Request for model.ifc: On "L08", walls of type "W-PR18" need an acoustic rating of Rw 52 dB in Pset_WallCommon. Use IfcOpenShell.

First a look at what the model holds.

```python
import ifcopenshell
import ifcopenshell.util.element

model = ifcopenshell.open("model.ifc")
print(model.schema)
storey = next(s for s in model.by_type("IfcBuildingStorey") if s.Name == "L08")
walls = [e for e in ifcopenshell.util.element.get_decomposition(storey) if e.is_a("IfcWall")]
seen = {}
for e in walls:
    element_type = ifcopenshell.util.element.get_type(e)
    key = (element_type.Name if element_type != e and element_type else None, ifcopenshell.util.element.get_pset(e, "Pset_WallCommon", "AcousticRating"))
    seen[key] = seen.get(key, 0) + 1
for (name, value), count in sorted(seen.items(), key=str):
    print(count, "x", name, "|", value)
```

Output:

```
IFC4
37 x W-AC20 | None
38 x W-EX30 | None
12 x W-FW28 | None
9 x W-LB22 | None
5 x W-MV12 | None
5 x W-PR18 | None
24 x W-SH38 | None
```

```python
import ifcopenshell
import ifcopenshell.api.pset
import ifcopenshell.util.element

model = ifcopenshell.open("model.ifc")

storey = next(s for s in model.by_type("IfcBuildingStorey") if s.Name == "L08")
walls = [e for e in ifcopenshell.util.element.get_decomposition(storey) if e.is_a("IfcWall")]

count = 0
for e in walls:
    element_type = ifcopenshell.util.element.get_type(e)
    if element_type in (None, e) or element_type.Name != "W-PR18":
        continue
    # add_pset returns the element's existing set when there is one.
    pset = ifcopenshell.api.pset.add_pset(model, product=e, name="Pset_WallCommon")
    ifcopenshell.api.pset.edit_pset(model, pset=pset, properties={"AcousticRating": "Rw 52 dB"})
    count += 1

print(count, "walls updated")

model.write("model_edited.ifc")
```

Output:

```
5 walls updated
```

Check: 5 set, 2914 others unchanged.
